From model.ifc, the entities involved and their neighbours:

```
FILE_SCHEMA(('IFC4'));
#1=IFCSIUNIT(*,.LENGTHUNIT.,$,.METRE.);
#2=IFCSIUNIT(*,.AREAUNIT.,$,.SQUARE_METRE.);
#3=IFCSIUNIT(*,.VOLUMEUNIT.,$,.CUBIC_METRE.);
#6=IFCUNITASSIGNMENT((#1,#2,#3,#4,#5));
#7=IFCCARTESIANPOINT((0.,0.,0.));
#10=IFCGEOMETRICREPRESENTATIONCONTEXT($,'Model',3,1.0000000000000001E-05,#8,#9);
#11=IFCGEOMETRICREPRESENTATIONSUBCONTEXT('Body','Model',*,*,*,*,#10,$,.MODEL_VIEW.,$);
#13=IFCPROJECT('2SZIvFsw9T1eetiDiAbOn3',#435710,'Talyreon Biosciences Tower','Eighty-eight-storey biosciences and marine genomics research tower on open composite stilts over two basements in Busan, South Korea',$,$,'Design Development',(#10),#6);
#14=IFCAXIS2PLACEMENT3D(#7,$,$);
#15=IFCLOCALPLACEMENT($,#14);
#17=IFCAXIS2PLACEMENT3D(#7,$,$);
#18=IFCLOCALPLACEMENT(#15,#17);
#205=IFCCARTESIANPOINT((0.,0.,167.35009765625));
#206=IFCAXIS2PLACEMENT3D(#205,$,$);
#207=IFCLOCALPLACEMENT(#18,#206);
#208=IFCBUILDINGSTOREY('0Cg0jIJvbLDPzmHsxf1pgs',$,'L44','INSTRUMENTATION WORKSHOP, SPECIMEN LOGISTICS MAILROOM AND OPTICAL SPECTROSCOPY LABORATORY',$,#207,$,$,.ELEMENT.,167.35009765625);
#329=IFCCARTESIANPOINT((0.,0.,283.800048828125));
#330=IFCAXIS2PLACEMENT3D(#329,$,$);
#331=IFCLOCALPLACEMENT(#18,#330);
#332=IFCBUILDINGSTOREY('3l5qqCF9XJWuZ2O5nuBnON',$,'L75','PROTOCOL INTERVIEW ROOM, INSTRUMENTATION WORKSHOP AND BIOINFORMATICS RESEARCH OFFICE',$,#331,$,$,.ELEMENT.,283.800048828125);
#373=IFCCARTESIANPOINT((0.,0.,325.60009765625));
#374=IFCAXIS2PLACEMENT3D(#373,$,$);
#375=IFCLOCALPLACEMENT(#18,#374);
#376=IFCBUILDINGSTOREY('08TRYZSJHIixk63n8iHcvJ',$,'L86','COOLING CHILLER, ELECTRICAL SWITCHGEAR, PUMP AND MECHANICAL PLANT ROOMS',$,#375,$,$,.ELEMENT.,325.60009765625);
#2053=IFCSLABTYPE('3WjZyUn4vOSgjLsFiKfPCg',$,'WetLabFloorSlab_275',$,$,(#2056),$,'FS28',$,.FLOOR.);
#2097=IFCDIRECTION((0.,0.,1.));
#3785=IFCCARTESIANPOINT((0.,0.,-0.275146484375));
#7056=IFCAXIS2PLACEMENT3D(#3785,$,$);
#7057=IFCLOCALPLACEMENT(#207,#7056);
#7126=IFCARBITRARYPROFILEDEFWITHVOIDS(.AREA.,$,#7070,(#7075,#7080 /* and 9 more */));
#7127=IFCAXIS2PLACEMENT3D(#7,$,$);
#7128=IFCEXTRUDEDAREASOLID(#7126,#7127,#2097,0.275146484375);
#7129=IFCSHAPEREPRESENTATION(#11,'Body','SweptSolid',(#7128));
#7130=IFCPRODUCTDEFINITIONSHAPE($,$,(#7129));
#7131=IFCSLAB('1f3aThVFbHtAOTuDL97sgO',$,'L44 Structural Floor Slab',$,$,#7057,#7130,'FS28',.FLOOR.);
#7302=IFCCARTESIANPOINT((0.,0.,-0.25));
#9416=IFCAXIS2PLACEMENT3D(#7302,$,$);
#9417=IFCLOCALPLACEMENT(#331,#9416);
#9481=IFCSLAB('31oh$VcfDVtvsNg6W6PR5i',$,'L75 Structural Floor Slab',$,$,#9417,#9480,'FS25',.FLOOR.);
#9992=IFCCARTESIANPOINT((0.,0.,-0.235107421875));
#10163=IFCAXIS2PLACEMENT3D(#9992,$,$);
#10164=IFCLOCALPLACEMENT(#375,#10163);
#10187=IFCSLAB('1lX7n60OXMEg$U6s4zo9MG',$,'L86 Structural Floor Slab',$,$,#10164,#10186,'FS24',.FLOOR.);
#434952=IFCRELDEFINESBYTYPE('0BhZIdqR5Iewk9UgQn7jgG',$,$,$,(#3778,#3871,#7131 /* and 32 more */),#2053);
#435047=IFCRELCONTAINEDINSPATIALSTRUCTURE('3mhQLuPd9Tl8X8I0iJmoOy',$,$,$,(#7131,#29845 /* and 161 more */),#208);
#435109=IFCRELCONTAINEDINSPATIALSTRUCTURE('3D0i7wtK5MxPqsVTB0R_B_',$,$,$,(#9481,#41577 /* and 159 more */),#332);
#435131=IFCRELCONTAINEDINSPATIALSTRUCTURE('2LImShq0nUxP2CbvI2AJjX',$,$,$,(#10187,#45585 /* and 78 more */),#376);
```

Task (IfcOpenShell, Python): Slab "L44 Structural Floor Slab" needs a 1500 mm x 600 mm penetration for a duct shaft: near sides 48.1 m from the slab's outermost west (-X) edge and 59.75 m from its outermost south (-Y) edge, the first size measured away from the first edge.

```python
import numpy as np
import ifcopenshell
import ifcopenshell.api.feature
import ifcopenshell.api.geometry
import ifcopenshell.api.root
import ifcopenshell.geom
import ifcopenshell.util.placement
import ifcopenshell.util.representation
import ifcopenshell.util.shape
import ifcopenshell.util.unit

model = ifcopenshell.open("model.ifc")
unit_scale = ifcopenshell.util.unit.calculate_unit_scale(model)
settings = ifcopenshell.geom.settings()


def volume(element):
    """Net volume in cubic metres, openings subtracted."""
    shape = ifcopenshell.geom.create_shape(settings, element)
    return ifcopenshell.util.shape.get_volume(shape.geometry)


slab = model.by_guid("1f3aThVFbHtAOTuDL97sgO")
before = volume(slab)

# Extent in the slab's own axes, in metres. The edges named are its -X and -Y sides.
slab_shape = ifcopenshell.geom.create_shape(settings, slab)
vertices = ifcopenshell.util.shape.get_vertices(slab_shape.geometry)
x_min, y_min, bottom = vertices.min(axis=0)
top = vertices[:, 2].max()

opening = ifcopenshell.api.root.create_entity(model, ifc_class="IfcOpeningElement", name="Duct shaft opening", predefined_type="OPENING")
context = ifcopenshell.util.representation.get_context(model, "Model", "Body", "MODEL_VIEW")
width, depth = 1.5, 0.6
outline = [(0.0, 0.0), (width, 0.0), (width, depth), (0.0, depth), (0.0, 0.0)]
# Overshoot both faces by 50 mm so the cut is clean.
shape = ifcopenshell.api.geometry.add_slab_representation(
    model, context=context, depth=top - bottom + 0.1, polyline=outline
)
ifcopenshell.api.geometry.assign_representation(model, product=opening, representation=shape)

matrix = ifcopenshell.util.placement.get_local_placement(slab.ObjectPlacement)
matrix[:, 3] = matrix @ np.append(np.array([x_min + 48.1, y_min + 59.75, bottom - 0.05]) / unit_scale, 1.0)
ifcopenshell.api.geometry.edit_object_placement(model, product=opening, matrix=matrix, is_si=False)
ifcopenshell.api.feature.add_feature(model, feature=opening, element=slab)

after = volume(slab)

print(f"slab volume {before:.3f} -> {after:.3f} m3")

model.write("model-out.ifc")
```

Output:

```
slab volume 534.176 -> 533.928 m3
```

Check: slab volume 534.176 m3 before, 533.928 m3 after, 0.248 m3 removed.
